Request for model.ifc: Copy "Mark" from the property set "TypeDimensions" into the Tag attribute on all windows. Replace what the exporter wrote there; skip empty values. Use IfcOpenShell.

First a look at what the model holds.

```python
import ifcopenshell
import ifcopenshell.util.element

model = ifcopenshell.open("model.ifc")
print(model.schema)
windows = model.by_type("IfcWindow")
print(len(windows), "windows")
for e in windows[:8]:
    source = ifcopenshell.util.element.get_pset(e, "TypeDimensions", "Mark")
    target = e.Tag
    print(e.id(), repr(source), repr(target), sep=" | ")
```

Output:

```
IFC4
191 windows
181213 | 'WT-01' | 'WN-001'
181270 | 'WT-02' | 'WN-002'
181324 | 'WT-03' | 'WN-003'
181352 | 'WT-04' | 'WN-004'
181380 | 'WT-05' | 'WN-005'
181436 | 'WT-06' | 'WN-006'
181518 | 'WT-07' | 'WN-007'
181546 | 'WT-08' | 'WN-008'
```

```python
import ifcopenshell
import ifcopenshell.util.element

model = ifcopenshell.open("model.ifc")

count = 0
for e in model.by_type("IfcWindow"):
    value = ifcopenshell.util.element.get_pset(e, "TypeDimensions", "Mark")
    current = e.Tag
    if not value or not value.strip() or current == value:
        continue
    e.Tag = value
    count += 1

print(count, "windows updated")

model.write("model_rev.ifc")
```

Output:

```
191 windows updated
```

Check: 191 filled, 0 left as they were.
